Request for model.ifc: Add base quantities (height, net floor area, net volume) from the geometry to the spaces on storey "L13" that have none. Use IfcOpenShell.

First a look at what the model holds.

```python
import ifcopenshell
import ifcopenshell.util.element
import ifcopenshell.util.unit

model = ifcopenshell.open("model.ifc")
print(model.schema)
for unit_type in ("LENGTHUNIT", "AREAUNIT", "VOLUMEUNIT"):
    print(unit_type, ifcopenshell.util.unit.calculate_unit_scale(model, unit_type))
storey = next(s for s in model.by_type("IfcBuildingStorey") if s.Name == "L13")
spaces = [e for e in ifcopenshell.util.element.get_decomposition(storey) if e.is_a("IfcSpace")]
for e in sorted(spaces, key=lambda e: e.id()):
    print(e.id(), e.is_a(), e.Name, list(ifcopenshell.util.element.get_psets(e, qtos_only=True)), sep=" | ")
```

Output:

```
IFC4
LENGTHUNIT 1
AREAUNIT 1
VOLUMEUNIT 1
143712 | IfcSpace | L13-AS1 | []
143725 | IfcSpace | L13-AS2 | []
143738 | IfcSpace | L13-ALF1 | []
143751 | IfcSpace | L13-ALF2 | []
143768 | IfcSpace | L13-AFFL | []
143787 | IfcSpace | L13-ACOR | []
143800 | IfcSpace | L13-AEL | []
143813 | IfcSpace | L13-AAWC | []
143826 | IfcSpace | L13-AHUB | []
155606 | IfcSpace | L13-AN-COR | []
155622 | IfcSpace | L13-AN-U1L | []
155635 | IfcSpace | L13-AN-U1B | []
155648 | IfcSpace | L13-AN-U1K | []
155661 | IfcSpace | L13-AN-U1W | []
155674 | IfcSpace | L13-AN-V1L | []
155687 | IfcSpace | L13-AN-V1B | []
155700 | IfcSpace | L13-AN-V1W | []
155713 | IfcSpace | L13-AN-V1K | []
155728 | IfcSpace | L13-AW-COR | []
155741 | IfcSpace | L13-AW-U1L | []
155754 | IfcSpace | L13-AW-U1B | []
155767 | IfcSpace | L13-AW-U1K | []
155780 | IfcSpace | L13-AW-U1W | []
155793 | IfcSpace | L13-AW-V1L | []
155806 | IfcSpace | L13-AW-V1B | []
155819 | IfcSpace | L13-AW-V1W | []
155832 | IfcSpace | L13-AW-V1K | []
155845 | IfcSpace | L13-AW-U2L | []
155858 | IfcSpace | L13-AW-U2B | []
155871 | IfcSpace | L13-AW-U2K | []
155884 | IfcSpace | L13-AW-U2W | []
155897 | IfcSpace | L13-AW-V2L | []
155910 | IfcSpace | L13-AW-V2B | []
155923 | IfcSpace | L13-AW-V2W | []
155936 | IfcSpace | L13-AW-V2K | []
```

```python
import ifcopenshell
import ifcopenshell.api.pset
import ifcopenshell.geom
import ifcopenshell.util.element
import ifcopenshell.util.shape
import ifcopenshell.util.unit

model = ifcopenshell.open("model.ifc")
unit_scale = ifcopenshell.util.unit.calculate_unit_scale(model)
area_scale = ifcopenshell.util.unit.calculate_unit_scale(model, "AREAUNIT")
volume_scale = ifcopenshell.util.unit.calculate_unit_scale(model, "VOLUMEUNIT")
settings = ifcopenshell.geom.settings()

storey = next(s for s in model.by_type("IfcBuildingStorey") if s.Name == "L13")
spaces = [e for e in ifcopenshell.util.element.get_decomposition(storey) if e.is_a("IfcSpace")]

for e in sorted(spaces, key=lambda e: e.id()):
    if ifcopenshell.util.element.get_psets(e, qtos_only=True, should_inherit=False):
        continue
    # Geometry comes back in metres, in the element's own axes.
    shape = ifcopenshell.geom.create_shape(settings, e)
    values = {
        "Height": ifcopenshell.util.shape.get_z(shape.geometry) / unit_scale,
        "NetFloorArea": ifcopenshell.util.shape.get_footprint_area(shape.geometry) / area_scale,
        "NetVolume": ifcopenshell.util.shape.get_volume(shape.geometry) / volume_scale,
    }
    qto = ifcopenshell.api.pset.add_qto(model, product=e, name="Qto_SpaceBaseQuantities")
    ifcopenshell.api.pset.edit_qto(model, qto=qto, properties=values)
    print(e.id(), {k: round(v, 3) for k, v in values.items()})

model.write("model_v2.ifc")
```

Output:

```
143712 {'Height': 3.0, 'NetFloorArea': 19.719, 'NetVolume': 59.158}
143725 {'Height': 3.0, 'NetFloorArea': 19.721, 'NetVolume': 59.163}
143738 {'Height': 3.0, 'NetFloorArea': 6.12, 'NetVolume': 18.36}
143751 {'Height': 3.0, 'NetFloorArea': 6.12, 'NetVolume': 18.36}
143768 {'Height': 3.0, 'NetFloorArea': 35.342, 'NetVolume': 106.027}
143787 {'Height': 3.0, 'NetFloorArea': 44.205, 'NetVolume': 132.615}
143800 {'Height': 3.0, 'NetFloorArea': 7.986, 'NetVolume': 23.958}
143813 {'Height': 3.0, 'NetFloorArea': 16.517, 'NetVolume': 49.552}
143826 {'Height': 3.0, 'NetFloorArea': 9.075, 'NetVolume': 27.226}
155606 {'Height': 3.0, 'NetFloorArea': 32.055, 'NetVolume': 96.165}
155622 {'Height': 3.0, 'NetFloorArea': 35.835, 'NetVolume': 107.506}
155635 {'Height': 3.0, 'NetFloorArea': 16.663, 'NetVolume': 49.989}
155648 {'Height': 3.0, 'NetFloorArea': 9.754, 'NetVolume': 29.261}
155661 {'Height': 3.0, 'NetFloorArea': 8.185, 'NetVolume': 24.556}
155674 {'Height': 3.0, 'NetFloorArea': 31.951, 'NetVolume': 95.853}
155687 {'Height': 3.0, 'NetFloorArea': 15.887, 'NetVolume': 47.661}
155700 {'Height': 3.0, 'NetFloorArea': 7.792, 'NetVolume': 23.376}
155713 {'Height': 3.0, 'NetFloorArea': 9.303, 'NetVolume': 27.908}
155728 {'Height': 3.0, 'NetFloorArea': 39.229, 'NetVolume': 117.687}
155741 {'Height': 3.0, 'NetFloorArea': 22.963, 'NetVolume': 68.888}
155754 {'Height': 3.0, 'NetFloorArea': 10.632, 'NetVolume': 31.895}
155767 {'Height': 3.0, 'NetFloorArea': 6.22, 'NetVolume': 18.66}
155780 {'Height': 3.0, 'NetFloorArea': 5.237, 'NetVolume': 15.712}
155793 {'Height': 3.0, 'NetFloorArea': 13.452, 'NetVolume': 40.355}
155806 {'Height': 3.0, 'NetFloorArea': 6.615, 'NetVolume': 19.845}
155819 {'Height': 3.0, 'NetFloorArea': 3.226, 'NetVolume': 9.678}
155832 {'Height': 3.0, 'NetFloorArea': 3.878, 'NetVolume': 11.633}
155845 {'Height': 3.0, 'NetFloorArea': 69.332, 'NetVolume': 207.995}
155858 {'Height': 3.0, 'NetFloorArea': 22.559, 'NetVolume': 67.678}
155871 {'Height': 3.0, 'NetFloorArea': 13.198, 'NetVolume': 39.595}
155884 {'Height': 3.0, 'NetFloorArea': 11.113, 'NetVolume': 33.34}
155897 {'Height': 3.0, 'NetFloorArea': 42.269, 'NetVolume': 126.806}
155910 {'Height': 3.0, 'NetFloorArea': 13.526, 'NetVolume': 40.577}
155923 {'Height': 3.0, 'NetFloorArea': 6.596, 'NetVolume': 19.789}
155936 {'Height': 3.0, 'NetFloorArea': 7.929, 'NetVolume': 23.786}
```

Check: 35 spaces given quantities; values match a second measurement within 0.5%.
